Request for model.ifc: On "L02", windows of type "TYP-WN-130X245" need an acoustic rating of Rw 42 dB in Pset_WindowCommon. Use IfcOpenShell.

First a look at what the model holds.

```python
import ifcopenshell
import ifcopenshell.util.element

model = ifcopenshell.open("model.ifc")
print(model.schema)
storey = next(s for s in model.by_type("IfcBuildingStorey") if s.Name == "L02")
windows = [e for e in ifcopenshell.util.element.get_decomposition(storey) if e.is_a("IfcWindow")]
seen = {}
for e in windows:
    element_type = ifcopenshell.util.element.get_type(e)
    key = (element_type.Name if element_type != e and element_type else None, ifcopenshell.util.element.get_pset(e, "Pset_WindowCommon", "AcousticRating"))
    seen[key] = seen.get(key, 0) + 1
for (name, value), count in sorted(seen.items(), key=str):
    print(count, "x", name, "|", value)
```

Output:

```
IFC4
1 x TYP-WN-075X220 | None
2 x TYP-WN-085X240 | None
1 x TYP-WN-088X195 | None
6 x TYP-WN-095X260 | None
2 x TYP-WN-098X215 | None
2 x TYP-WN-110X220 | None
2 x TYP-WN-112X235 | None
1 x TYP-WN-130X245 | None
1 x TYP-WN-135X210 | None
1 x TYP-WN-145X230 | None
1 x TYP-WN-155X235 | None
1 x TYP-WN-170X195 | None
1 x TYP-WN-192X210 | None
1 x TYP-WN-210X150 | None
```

```python
import ifcopenshell
import ifcopenshell.api.pset
import ifcopenshell.util.element

model = ifcopenshell.open("model.ifc")

storey = next(s for s in model.by_type("IfcBuildingStorey") if s.Name == "L02")
windows = [e for e in ifcopenshell.util.element.get_decomposition(storey) if e.is_a("IfcWindow")]

count = 0
for e in windows:
    element_type = ifcopenshell.util.element.get_type(e)
    if element_type in (None, e) or element_type.Name != "TYP-WN-130X245":
        continue
    # add_pset returns the element's existing set when there is one.
    pset = ifcopenshell.api.pset.add_pset(model, product=e, name="Pset_WindowCommon")
    ifcopenshell.api.pset.edit_pset(model, pset=pset, properties={"AcousticRating": "Rw 42 dB"})
    count += 1

print(count, "windows updated")

model.write("model_v2.ifc")
```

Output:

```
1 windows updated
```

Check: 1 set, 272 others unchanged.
